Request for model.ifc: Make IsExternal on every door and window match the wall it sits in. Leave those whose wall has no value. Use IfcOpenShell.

First a look at what the model holds.

```python
import ifcopenshell
import ifcopenshell.util.element

model = ifcopenshell.open("model.ifc")
print(model.schema)
seen = {}
for e in model.by_type("IfcDoor") + model.by_type("IfcWindow"):
    if not e.FillsVoids:
        continue
    host = e.FillsVoids[0].RelatingOpeningElement.VoidsElements[0].RelatingBuildingElement
    own = ifcopenshell.util.element.get_pset(e, f"Pset_{e.is_a()[3:].removesuffix('StandardCase')}Common", "IsExternal")
    wall = ifcopenshell.util.element.get_pset(host, "Pset_WallCommon", "IsExternal")
    seen[e.is_a(), own, wall] = seen.get((e.is_a(), own, wall), 0) + 1
for (cls, own, wall), count in sorted(seen.items(), key=str):
    print(count, cls, "IsExternal:", own, "| host wall:", wall)
```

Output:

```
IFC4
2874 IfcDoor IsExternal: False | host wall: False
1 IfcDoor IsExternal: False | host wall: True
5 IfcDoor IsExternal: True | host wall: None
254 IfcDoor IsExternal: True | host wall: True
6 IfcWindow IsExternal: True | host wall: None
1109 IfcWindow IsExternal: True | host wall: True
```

```python
import ifcopenshell
import ifcopenshell.api.pset
import ifcopenshell.util.element

model = ifcopenshell.open("model.ifc")

count = 0
for ifc_class, pset_name in (("IfcDoor", "Pset_DoorCommon"), ("IfcWindow", "Pset_WindowCommon")):
    for e in model.by_type(ifc_class):
        if not e.FillsVoids:
            continue
        host = e.FillsVoids[0].RelatingOpeningElement.VoidsElements[0].RelatingBuildingElement
        external = ifcopenshell.util.element.get_pset(host, "Pset_WallCommon", "IsExternal")
        if external is None or ifcopenshell.util.element.get_pset(e, pset_name, "IsExternal") == external:
            continue
        found = ifcopenshell.util.element.get_pset(e, pset_name, should_inherit=False)
        if found:
            pset = model.by_id(found["id"])
            if len(ifcopenshell.util.element.get_elements_by_pset(pset)) > 1:
                pset = ifcopenshell.api.pset.unshare_pset(model, products=[e], pset=pset)[0]
        else:
            pset = ifcopenshell.api.pset.add_pset(model, product=e, name=pset_name)
        ifcopenshell.api.pset.edit_pset(model, pset=pset, properties={"IsExternal": external})
        count += 1

print(count, "updated")

model.write("model_rev.ifc")
```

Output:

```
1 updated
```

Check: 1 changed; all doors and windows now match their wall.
